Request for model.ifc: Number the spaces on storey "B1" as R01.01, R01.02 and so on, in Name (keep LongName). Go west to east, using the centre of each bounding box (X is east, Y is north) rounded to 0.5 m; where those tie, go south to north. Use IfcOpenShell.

First a look at what the model holds.

```python
import ifcopenshell
import ifcopenshell.util.element
import ifcopenshell.util.placement

model = ifcopenshell.open("model.ifc")
print(model.schema)
storey = next(s for s in model.by_type("IfcBuildingStorey") if s.Name == "B1")
spaces = [e for e in ifcopenshell.util.element.get_decomposition(storey) if e.is_a("IfcSpace")]
for e in sorted(spaces, key=lambda e: e.id()):
    origin = ifcopenshell.util.placement.get_local_placement(e.ObjectPlacement)[:3, 3]
    print(e.id(), e.Name, e.LongName, origin.round(2) + 0.0, sep=" | ")
```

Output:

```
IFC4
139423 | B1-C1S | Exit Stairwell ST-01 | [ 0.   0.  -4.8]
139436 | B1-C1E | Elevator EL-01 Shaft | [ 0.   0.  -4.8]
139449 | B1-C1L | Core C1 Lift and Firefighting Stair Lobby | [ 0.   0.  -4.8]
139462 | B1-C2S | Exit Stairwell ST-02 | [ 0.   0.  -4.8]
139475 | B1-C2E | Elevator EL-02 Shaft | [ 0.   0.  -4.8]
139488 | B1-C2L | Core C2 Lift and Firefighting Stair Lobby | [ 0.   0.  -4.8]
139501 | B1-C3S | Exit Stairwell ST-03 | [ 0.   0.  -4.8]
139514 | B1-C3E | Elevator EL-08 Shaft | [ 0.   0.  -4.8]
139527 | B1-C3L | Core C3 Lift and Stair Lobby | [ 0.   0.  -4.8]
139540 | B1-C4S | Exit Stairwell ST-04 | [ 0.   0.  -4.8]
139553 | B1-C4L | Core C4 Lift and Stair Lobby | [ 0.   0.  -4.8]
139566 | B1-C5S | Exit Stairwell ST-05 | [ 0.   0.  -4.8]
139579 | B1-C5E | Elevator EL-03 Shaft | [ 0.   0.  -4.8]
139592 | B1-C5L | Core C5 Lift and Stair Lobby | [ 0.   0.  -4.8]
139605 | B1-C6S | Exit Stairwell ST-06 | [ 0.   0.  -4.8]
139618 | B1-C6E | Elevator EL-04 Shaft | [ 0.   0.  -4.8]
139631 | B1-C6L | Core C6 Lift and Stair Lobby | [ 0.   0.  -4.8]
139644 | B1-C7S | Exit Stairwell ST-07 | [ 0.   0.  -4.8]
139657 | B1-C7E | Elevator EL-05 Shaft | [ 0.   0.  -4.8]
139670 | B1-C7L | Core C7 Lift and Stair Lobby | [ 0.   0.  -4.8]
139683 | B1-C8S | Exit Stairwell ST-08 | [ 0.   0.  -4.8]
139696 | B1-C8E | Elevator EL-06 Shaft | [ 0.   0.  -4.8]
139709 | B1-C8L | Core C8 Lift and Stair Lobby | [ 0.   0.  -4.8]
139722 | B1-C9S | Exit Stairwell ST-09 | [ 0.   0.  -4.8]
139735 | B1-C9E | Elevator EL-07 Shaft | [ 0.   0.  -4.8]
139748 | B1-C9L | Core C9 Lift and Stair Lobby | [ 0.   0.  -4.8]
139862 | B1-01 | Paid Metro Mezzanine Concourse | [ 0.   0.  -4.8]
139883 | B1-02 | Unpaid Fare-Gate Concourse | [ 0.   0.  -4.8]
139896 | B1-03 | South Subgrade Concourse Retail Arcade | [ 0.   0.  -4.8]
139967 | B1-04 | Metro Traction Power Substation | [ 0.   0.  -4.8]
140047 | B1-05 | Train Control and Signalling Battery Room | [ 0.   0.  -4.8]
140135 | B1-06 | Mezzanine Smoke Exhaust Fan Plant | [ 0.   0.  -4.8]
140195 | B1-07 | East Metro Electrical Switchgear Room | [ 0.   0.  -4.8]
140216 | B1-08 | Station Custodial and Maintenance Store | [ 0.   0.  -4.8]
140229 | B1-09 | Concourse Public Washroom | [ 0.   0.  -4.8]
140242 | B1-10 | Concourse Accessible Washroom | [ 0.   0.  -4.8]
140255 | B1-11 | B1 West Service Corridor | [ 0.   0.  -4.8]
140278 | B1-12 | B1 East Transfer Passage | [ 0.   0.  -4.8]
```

```python
import ifcopenshell
import ifcopenshell.geom
import ifcopenshell.util.element
import ifcopenshell.util.shape

model = ifcopenshell.open("model.ifc")
settings = ifcopenshell.geom.settings()
settings.set("use-world-coords", True)


def centre(element):
    shape = ifcopenshell.geom.create_shape(settings, element)
    return ifcopenshell.util.shape.get_bbox_centroid(shape.geometry)


storey = next(s for s in model.by_type("IfcBuildingStorey") if s.Name == "B1")
spaces = [e for e in ifcopenshell.util.element.get_decomposition(storey) if e.is_a("IfcSpace")]

# Insertion points can sit at a corner or the storey origin, so sort by the geometry (in metres).
centres = {e: centre(e) for e in spaces}
spaces.sort(key=lambda e: (round(centres[e][0] / 0.5), centres[e][1]))

for i, e in enumerate(spaces, start=1):
    number = f"R01.{i:02d}"
    e.Name = number
    print(e.id(), number)

model.write("model_rev.ifc")
```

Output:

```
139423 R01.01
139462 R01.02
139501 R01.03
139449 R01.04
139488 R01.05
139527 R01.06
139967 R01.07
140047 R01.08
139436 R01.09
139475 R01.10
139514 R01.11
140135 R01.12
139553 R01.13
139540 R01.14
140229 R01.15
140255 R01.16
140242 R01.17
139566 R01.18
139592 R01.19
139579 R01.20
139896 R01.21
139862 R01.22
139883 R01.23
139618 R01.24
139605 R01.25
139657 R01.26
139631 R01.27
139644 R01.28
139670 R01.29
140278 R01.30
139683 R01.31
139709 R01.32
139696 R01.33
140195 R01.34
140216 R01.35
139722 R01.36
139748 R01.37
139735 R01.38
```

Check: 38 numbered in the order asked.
